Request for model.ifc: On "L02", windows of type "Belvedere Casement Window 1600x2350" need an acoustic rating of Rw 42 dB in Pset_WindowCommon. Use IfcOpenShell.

First a look at what the model holds.

```python
import ifcopenshell
import ifcopenshell.util.element

model = ifcopenshell.open("model.ifc")
print(model.schema)
storey = next(s for s in model.by_type("IfcBuildingStorey") if s.Name == "L02")
windows = [e for e in ifcopenshell.util.element.get_decomposition(storey) if e.is_a("IfcWindow")]
seen = {}
for e in windows:
    element_type = ifcopenshell.util.element.get_type(e)
    key = (element_type.Name if element_type != e and element_type else None, ifcopenshell.util.element.get_pset(e, "Pset_WindowCommon", "AcousticRating"))
    seen[key] = seen.get(key, 0) + 1
for (name, value), count in sorted(seen.items(), key=str):
    print(count, "x", name, "|", value)
```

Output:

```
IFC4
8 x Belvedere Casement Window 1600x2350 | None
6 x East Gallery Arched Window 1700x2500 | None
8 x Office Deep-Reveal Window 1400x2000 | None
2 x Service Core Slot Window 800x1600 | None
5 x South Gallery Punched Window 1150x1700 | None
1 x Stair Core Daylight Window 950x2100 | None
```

```python
import ifcopenshell
import ifcopenshell.api.pset
import ifcopenshell.util.element

model = ifcopenshell.open("model.ifc")

storey = next(s for s in model.by_type("IfcBuildingStorey") if s.Name == "L02")
windows = [e for e in ifcopenshell.util.element.get_decomposition(storey) if e.is_a("IfcWindow")]

count = 0
for e in windows:
    element_type = ifcopenshell.util.element.get_type(e)
    if element_type in (None, e) or element_type.Name != "Belvedere Casement Window 1600x2350":
        continue
    # add_pset returns the element's existing set when there is one.
    pset = ifcopenshell.api.pset.add_pset(model, product=e, name="Pset_WindowCommon")
    ifcopenshell.api.pset.edit_pset(model, pset=pset, properties={"AcousticRating": "Rw 42 dB"})
    count += 1

print(count, "windows updated")

model.write("model_rev.ifc")
```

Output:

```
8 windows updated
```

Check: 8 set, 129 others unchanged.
